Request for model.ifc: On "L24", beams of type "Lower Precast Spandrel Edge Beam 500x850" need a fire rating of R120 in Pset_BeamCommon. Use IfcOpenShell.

First a look at what the model holds.

```python
import ifcopenshell
import ifcopenshell.util.element

model = ifcopenshell.open("model.ifc")
print(model.schema)
storey = next(s for s in model.by_type("IfcBuildingStorey") if s.Name == "L24")
beams = [e for e in ifcopenshell.util.element.get_decomposition(storey) if e.is_a("IfcBeam")]
seen = {}
for e in beams:
    element_type = ifcopenshell.util.element.get_type(e)
    key = (element_type.Name if element_type != e and element_type else None, ifcopenshell.util.element.get_pset(e, "Pset_BeamCommon", "FireRating"))
    seen[key] = seen.get(key, 0) + 1
for (name, value), count in sorted(seen.items(), key=str):
    print(count, "x", name, "|", value)
```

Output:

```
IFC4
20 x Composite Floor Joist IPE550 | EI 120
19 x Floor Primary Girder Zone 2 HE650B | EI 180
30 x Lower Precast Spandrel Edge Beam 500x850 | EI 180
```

```python
import ifcopenshell
import ifcopenshell.api.pset
import ifcopenshell.util.element

model = ifcopenshell.open("model.ifc")

storey = next(s for s in model.by_type("IfcBuildingStorey") if s.Name == "L24")
beams = [e for e in ifcopenshell.util.element.get_decomposition(storey) if e.is_a("IfcBeam")]

count = 0
for e in beams:
    element_type = ifcopenshell.util.element.get_type(e)
    if element_type in (None, e) or element_type.Name != "Lower Precast Spandrel Edge Beam 500x850":
        continue
    # add_pset returns the element's existing set when there is one.
    pset = ifcopenshell.api.pset.add_pset(model, product=e, name="Pset_BeamCommon")
    ifcopenshell.api.pset.edit_pset(model, pset=pset, properties={"FireRating": "R120"})
    count += 1

print(count, "beams updated")

model.write("model-out.ifc")
```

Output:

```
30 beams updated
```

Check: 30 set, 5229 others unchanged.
